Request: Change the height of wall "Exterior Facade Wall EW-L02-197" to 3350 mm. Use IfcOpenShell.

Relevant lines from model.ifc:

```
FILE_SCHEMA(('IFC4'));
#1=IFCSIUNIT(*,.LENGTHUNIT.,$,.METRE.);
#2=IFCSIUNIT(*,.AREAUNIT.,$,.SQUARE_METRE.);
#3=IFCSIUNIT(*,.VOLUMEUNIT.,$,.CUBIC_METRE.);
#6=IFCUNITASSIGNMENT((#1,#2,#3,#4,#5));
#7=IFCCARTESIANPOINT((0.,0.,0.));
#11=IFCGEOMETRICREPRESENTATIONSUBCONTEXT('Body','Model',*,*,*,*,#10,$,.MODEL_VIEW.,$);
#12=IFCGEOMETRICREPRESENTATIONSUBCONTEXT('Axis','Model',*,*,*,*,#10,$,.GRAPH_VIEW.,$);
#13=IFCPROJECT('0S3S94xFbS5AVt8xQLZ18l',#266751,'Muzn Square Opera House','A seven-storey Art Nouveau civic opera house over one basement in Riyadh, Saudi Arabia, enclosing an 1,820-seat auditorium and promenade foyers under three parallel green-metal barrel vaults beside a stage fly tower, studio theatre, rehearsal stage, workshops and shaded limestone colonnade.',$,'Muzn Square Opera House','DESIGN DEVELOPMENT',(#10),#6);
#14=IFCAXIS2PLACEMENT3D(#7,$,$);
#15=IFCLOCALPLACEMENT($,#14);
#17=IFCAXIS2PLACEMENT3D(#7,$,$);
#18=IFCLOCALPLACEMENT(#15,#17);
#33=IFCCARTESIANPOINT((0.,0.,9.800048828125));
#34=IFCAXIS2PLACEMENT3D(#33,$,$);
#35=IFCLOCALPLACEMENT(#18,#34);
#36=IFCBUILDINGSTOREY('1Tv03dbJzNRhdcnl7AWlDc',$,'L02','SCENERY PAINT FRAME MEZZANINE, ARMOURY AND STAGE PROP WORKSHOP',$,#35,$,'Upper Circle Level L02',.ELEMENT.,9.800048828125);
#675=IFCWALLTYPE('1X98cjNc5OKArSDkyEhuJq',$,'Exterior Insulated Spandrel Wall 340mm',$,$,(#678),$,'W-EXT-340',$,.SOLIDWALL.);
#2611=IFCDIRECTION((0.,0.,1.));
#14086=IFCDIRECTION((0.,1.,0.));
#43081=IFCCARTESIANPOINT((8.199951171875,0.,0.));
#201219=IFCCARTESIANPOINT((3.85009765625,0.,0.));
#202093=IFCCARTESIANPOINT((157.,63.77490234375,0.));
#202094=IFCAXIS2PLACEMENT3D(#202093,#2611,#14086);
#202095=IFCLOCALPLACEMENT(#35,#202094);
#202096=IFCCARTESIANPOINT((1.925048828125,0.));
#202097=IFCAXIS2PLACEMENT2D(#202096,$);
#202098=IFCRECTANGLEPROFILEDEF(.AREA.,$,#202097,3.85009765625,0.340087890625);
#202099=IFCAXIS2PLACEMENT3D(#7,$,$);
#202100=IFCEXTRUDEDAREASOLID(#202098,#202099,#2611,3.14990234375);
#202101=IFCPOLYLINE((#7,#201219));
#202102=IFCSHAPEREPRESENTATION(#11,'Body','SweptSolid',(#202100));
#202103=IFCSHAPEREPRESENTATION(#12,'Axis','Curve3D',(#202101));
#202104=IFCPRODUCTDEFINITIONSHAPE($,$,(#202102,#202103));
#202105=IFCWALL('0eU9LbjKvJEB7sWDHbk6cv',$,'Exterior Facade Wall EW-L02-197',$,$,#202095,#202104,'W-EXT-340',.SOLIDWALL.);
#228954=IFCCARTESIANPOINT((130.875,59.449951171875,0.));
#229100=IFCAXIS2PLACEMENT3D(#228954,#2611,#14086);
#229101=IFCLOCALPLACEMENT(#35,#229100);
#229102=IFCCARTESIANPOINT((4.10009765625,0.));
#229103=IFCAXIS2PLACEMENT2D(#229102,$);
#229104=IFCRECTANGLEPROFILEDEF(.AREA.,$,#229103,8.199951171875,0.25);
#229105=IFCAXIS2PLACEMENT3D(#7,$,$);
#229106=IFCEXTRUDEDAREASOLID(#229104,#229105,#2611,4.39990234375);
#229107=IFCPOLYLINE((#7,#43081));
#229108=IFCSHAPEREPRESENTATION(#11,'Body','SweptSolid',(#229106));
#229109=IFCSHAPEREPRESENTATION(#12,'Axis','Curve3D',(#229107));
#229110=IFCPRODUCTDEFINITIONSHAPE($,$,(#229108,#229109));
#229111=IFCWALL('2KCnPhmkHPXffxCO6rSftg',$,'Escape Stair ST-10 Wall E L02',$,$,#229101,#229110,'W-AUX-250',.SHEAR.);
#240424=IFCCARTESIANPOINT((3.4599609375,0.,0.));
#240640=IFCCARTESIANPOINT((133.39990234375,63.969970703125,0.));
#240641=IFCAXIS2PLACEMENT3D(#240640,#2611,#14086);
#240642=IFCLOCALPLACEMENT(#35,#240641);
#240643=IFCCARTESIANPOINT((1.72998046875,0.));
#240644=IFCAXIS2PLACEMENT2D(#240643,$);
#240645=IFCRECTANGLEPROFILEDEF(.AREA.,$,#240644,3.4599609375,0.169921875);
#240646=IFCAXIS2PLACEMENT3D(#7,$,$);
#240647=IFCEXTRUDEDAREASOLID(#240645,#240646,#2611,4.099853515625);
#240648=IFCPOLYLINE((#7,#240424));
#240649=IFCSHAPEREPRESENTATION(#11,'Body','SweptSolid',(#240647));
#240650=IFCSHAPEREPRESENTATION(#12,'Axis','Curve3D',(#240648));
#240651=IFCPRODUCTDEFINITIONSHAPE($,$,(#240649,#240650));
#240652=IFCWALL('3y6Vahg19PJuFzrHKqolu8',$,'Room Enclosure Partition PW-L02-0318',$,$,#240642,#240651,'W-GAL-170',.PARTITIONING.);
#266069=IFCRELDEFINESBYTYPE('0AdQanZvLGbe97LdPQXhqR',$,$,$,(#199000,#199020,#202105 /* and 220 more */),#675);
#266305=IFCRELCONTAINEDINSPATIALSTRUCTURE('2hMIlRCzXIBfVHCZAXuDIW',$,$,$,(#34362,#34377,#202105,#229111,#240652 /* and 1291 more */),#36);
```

```python
import ifcopenshell
import ifcopenshell.geom
import ifcopenshell.util.representation
import ifcopenshell.util.shape
import ifcopenshell.util.unit

model = ifcopenshell.open("model.ifc")
unit_scale = ifcopenshell.util.unit.calculate_unit_scale(model)
settings = ifcopenshell.geom.settings()


def volume(element):
    """Net volume in cubic metres, openings subtracted."""
    shape = ifcopenshell.geom.create_shape(settings, element)
    return ifcopenshell.util.shape.get_volume(shape.geometry)


wall = model.by_id(202105)
before = volume(wall)

body = ifcopenshell.util.representation.get_representation(wall, "Model", "Body")
solid = body.Items[0]
old_height = solid.Depth
solid.Depth = 3.35 / unit_scale
after = volume(wall)

print(f"height {old_height:g} -> {solid.Depth:g}, volume {before:.3f} -> {after:.3f} m3")

model.write("model_v2.ifc")
```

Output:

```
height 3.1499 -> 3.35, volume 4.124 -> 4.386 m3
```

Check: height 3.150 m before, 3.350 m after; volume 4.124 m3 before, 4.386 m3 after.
